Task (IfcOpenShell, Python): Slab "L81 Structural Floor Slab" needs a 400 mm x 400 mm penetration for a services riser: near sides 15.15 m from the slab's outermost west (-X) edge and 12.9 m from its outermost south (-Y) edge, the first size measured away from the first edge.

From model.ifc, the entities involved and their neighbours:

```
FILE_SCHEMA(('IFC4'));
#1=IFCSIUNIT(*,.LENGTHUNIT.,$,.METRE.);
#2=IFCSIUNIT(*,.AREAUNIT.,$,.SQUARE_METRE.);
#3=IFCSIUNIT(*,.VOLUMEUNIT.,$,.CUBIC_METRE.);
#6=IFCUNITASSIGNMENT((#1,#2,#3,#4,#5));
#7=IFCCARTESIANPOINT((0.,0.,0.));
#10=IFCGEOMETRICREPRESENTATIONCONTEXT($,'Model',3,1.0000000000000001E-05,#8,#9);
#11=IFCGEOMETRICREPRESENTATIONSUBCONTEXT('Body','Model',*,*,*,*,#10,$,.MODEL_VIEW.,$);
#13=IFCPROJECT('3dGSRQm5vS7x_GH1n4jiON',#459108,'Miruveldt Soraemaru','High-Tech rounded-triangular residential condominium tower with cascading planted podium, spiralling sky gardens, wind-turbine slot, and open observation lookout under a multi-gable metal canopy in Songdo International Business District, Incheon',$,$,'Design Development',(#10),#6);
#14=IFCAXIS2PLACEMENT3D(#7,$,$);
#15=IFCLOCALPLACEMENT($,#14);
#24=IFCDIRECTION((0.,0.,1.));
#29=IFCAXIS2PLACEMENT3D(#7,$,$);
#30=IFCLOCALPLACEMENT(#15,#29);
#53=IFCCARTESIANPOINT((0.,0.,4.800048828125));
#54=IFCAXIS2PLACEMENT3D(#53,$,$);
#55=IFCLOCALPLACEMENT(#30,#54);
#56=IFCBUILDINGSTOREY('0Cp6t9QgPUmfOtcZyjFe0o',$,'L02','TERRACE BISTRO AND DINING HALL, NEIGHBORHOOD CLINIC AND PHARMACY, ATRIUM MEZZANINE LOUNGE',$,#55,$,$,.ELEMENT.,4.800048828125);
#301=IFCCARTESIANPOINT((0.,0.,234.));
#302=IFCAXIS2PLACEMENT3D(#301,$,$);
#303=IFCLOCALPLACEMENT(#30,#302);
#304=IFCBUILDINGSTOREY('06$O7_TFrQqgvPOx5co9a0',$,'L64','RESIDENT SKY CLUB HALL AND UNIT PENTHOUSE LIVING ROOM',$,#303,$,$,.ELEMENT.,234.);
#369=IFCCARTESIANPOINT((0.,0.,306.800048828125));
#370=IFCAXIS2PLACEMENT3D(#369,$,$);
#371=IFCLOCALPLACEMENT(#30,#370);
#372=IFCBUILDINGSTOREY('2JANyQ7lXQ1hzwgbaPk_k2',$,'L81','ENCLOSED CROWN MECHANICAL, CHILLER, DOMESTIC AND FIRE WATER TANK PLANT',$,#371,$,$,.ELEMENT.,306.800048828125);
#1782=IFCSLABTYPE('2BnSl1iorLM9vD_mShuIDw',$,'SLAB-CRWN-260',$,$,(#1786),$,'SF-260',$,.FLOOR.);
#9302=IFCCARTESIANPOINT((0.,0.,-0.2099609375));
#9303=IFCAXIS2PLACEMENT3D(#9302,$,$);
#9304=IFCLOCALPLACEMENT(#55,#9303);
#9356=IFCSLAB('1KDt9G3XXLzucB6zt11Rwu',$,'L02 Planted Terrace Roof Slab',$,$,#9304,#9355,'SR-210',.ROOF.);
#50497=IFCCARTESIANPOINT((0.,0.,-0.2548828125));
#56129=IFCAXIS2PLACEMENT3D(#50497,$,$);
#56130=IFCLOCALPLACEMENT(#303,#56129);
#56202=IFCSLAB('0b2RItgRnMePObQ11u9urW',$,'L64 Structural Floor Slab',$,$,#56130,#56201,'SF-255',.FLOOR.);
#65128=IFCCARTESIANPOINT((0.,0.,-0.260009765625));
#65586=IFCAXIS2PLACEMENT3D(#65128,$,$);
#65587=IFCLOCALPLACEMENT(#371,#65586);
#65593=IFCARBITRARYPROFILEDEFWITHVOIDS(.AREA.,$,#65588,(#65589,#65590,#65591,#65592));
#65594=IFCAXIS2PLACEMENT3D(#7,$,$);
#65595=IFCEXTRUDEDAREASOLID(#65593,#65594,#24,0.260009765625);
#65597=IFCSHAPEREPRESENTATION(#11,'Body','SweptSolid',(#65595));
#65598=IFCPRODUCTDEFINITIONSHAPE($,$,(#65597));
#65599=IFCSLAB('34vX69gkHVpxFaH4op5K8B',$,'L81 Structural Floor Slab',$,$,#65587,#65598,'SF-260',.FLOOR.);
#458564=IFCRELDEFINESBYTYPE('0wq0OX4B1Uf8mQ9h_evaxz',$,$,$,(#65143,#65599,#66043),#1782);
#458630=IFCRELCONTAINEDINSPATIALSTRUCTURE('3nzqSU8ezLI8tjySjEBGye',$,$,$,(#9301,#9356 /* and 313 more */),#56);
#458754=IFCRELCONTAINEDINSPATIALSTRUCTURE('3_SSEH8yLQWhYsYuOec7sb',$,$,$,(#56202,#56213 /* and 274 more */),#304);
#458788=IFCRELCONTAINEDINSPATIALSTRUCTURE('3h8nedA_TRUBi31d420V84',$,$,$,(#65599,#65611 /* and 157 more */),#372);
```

```python
import numpy as np
import ifcopenshell
import ifcopenshell.api.feature
import ifcopenshell.api.geometry
import ifcopenshell.api.root
import ifcopenshell.geom
import ifcopenshell.util.placement
import ifcopenshell.util.representation
import ifcopenshell.util.shape
import ifcopenshell.util.unit

model = ifcopenshell.open("model.ifc")
unit_scale = ifcopenshell.util.unit.calculate_unit_scale(model)
settings = ifcopenshell.geom.settings()


def volume(element):
    """Net volume in cubic metres, openings subtracted."""
    shape = ifcopenshell.geom.create_shape(settings, element)
    return ifcopenshell.util.shape.get_volume(shape.geometry)


slab = model.by_id(65599)
before = volume(slab)

# Extent in the slab's own axes, in metres. The edges named are its -X and -Y sides.
slab_shape = ifcopenshell.geom.create_shape(settings, slab)
vertices = ifcopenshell.util.shape.get_vertices(slab_shape.geometry)
x_min, y_min, bottom = vertices.min(axis=0)
top = vertices[:, 2].max()

opening = ifcopenshell.api.root.create_entity(model, ifc_class="IfcOpeningElement", name="Services riser opening", predefined_type="OPENING")
context = ifcopenshell.util.representation.get_context(model, "Model", "Body", "MODEL_VIEW")
width, depth = 0.4, 0.4
outline = [(0.0, 0.0), (width, 0.0), (width, depth), (0.0, depth), (0.0, 0.0)]
# Overshoot both faces by 50 mm so the cut is clean.
shape = ifcopenshell.api.geometry.add_slab_representation(
    model, context=context, depth=top - bottom + 0.1, polyline=outline
)
ifcopenshell.api.geometry.assign_representation(model, product=opening, representation=shape)

matrix = ifcopenshell.util.placement.get_local_placement(slab.ObjectPlacement)
matrix[:, 3] = matrix @ np.append(np.array([x_min + 15.15, y_min + 12.9, bottom - 0.05]) / unit_scale, 1.0)
ifcopenshell.api.geometry.edit_object_placement(model, product=opening, matrix=matrix, is_si=False)
ifcopenshell.api.feature.add_feature(model, feature=opening, element=slab)

after = volume(slab)

print(f"slab volume {before:.3f} -> {after:.3f} m3")

model.write("model_v2.ifc")
```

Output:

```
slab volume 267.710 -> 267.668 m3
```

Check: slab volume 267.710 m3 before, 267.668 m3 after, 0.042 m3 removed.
